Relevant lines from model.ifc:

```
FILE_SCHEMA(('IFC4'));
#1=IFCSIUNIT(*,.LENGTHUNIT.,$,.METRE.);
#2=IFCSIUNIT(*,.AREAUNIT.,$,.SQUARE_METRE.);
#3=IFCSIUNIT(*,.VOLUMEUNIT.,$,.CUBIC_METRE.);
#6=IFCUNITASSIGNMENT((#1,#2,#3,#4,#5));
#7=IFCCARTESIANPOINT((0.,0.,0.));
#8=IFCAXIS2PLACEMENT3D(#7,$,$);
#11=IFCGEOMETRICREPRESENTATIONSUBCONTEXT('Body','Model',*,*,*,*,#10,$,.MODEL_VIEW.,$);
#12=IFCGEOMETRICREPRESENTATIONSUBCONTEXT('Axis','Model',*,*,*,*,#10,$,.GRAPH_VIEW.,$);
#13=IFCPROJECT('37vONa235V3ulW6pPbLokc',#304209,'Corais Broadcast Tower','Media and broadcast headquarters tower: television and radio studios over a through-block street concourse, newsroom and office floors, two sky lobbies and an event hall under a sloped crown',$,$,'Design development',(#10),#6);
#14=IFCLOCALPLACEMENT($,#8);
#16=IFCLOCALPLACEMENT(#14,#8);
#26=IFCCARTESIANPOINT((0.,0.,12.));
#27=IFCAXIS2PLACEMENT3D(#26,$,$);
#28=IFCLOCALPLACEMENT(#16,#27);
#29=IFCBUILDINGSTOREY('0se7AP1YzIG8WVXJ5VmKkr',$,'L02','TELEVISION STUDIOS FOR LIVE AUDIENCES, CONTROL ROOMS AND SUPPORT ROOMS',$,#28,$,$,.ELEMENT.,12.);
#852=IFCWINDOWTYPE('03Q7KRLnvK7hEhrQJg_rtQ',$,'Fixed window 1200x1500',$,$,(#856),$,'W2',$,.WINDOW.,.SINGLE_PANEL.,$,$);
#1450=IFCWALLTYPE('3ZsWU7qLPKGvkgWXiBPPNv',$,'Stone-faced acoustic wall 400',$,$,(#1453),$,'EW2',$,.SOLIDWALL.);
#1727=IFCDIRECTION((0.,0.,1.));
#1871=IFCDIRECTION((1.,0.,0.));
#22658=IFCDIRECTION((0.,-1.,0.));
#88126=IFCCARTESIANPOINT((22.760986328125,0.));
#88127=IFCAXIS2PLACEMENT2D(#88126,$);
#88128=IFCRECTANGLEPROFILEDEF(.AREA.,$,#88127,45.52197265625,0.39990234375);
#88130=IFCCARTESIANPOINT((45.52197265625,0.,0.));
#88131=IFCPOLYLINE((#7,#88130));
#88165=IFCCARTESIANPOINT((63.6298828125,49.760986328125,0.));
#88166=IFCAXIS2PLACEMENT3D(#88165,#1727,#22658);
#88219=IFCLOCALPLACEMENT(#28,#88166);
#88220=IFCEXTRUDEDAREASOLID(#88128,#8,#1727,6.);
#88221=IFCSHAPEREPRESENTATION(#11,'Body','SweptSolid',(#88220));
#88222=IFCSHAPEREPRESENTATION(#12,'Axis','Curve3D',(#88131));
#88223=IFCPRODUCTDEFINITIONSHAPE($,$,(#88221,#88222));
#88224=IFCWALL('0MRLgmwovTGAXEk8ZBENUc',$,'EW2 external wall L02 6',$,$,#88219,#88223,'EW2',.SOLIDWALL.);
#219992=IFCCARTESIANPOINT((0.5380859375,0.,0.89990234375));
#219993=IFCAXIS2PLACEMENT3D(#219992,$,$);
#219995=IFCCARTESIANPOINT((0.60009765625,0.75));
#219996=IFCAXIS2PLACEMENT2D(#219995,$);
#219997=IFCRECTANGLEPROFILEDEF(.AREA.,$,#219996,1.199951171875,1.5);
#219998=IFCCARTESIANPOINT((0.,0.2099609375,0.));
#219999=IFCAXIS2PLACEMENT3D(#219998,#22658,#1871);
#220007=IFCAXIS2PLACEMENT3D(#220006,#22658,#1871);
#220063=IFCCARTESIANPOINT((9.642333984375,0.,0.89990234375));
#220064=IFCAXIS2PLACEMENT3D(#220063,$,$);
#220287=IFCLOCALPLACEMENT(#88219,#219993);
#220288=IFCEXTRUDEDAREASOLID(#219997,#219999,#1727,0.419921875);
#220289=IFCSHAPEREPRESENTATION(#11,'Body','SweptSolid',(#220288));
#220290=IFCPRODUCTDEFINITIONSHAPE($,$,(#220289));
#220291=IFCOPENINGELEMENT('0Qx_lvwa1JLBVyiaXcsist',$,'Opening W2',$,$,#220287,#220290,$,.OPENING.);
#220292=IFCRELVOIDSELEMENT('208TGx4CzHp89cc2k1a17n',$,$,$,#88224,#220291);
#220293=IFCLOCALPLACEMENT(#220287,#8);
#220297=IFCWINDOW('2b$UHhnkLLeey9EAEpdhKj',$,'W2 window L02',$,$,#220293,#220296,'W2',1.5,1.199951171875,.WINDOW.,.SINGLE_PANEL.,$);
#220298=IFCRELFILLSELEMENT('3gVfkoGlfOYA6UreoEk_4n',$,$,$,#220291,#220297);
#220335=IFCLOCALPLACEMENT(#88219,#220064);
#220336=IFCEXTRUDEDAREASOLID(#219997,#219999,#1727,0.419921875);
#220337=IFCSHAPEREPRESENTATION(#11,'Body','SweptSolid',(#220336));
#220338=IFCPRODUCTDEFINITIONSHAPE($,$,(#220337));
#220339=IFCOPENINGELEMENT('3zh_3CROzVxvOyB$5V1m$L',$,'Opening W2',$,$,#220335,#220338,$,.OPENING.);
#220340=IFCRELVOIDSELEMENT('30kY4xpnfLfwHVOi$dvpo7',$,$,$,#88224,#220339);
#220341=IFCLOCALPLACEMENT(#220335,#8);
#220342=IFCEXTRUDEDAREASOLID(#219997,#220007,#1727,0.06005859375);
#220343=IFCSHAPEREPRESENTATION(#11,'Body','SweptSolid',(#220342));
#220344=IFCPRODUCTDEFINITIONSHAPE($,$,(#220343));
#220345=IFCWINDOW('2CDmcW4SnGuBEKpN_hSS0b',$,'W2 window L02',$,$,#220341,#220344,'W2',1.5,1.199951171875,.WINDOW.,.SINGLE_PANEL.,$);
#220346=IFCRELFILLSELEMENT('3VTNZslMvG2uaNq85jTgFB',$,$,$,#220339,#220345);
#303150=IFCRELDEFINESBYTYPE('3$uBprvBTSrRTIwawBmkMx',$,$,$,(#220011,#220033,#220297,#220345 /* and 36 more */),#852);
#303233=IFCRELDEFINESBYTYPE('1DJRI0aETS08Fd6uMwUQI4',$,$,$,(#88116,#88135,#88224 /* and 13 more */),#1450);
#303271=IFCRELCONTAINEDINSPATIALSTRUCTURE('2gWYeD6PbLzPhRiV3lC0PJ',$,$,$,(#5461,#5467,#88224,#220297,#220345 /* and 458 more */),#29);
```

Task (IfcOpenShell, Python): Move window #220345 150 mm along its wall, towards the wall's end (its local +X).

```python
import ifcopenshell
import ifcopenshell.api.geometry
import ifcopenshell.util.placement
import ifcopenshell.util.unit

model = ifcopenshell.open("model.ifc")
unit_scale = ifcopenshell.util.unit.calculate_unit_scale(model)

window = model.by_guid("2CDmcW4SnGuBEKpN_hSS0b")
opening = window.FillsVoids[0].RelatingOpeningElement
wall = opening.VoidsElements[0].RelatingBuildingElement

wall_matrix = ifcopenshell.util.placement.get_local_placement(wall.ObjectPlacement)
shift = wall_matrix[:3, 0] * 0.15 / unit_scale
before = ifcopenshell.util.placement.get_local_placement(window.ObjectPlacement)[:3, 3].copy()

# The window is placed relative to its opening, so it follows when the opening moves.
matrix = ifcopenshell.util.placement.get_local_placement(opening.ObjectPlacement)
matrix[:3, 3] += shift
ifcopenshell.api.geometry.edit_object_placement(
    model, product=opening, matrix=matrix, is_si=False, should_transform_children=True
)

after = ifcopenshell.util.placement.get_local_placement(window.ObjectPlacement)[:3, 3]
print("window moved by", (after - before).round(3) + 0.0)

model.write("model-out.ifc")
```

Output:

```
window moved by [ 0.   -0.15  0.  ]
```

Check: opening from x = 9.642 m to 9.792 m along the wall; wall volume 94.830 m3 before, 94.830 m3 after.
